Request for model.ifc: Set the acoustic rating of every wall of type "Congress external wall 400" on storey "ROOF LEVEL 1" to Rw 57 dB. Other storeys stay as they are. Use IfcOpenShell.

First a look at what the model holds.

```python
import ifcopenshell
import ifcopenshell.util.element

model = ifcopenshell.open("model.ifc")
print(model.schema)
storey = next(s for s in model.by_type("IfcBuildingStorey") if s.Name == "ROOF LEVEL 1")
walls = [e for e in ifcopenshell.util.element.get_decomposition(storey) if e.is_a("IfcWall")]
seen = {}
for e in walls:
    element_type = ifcopenshell.util.element.get_type(e)
    key = (element_type.Name if element_type != e and element_type else None, ifcopenshell.util.element.get_pset(e, "Pset_WallCommon", "AcousticRating"))
    seen[key] = seen.get(key, 0) + 1
for (name, value), count in sorted(seen.items(), key=str):
    print(count, "x", name, "|", value)
```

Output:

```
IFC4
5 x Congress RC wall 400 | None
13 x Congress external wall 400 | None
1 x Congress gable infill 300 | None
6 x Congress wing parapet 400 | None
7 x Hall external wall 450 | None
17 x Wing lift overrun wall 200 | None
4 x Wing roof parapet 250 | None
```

```python
import ifcopenshell
import ifcopenshell.api.pset
import ifcopenshell.util.element

model = ifcopenshell.open("model.ifc")

storey = next(s for s in model.by_type("IfcBuildingStorey") if s.Name == "ROOF LEVEL 1")
walls = [e for e in ifcopenshell.util.element.get_decomposition(storey) if e.is_a("IfcWall")]

count = 0
for e in walls:
    element_type = ifcopenshell.util.element.get_type(e)
    if element_type in (None, e) or element_type.Name != "Congress external wall 400":
        continue
    # add_pset returns the element's existing set when there is one.
    pset = ifcopenshell.api.pset.add_pset(model, product=e, name="Pset_WallCommon")
    ifcopenshell.api.pset.edit_pset(model, pset=pset, properties={"AcousticRating": "Rw 57 dB"})
    count += 1

print(count, "walls updated")

model.write("model_updated.ifc")
```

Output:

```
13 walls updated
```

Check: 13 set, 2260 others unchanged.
